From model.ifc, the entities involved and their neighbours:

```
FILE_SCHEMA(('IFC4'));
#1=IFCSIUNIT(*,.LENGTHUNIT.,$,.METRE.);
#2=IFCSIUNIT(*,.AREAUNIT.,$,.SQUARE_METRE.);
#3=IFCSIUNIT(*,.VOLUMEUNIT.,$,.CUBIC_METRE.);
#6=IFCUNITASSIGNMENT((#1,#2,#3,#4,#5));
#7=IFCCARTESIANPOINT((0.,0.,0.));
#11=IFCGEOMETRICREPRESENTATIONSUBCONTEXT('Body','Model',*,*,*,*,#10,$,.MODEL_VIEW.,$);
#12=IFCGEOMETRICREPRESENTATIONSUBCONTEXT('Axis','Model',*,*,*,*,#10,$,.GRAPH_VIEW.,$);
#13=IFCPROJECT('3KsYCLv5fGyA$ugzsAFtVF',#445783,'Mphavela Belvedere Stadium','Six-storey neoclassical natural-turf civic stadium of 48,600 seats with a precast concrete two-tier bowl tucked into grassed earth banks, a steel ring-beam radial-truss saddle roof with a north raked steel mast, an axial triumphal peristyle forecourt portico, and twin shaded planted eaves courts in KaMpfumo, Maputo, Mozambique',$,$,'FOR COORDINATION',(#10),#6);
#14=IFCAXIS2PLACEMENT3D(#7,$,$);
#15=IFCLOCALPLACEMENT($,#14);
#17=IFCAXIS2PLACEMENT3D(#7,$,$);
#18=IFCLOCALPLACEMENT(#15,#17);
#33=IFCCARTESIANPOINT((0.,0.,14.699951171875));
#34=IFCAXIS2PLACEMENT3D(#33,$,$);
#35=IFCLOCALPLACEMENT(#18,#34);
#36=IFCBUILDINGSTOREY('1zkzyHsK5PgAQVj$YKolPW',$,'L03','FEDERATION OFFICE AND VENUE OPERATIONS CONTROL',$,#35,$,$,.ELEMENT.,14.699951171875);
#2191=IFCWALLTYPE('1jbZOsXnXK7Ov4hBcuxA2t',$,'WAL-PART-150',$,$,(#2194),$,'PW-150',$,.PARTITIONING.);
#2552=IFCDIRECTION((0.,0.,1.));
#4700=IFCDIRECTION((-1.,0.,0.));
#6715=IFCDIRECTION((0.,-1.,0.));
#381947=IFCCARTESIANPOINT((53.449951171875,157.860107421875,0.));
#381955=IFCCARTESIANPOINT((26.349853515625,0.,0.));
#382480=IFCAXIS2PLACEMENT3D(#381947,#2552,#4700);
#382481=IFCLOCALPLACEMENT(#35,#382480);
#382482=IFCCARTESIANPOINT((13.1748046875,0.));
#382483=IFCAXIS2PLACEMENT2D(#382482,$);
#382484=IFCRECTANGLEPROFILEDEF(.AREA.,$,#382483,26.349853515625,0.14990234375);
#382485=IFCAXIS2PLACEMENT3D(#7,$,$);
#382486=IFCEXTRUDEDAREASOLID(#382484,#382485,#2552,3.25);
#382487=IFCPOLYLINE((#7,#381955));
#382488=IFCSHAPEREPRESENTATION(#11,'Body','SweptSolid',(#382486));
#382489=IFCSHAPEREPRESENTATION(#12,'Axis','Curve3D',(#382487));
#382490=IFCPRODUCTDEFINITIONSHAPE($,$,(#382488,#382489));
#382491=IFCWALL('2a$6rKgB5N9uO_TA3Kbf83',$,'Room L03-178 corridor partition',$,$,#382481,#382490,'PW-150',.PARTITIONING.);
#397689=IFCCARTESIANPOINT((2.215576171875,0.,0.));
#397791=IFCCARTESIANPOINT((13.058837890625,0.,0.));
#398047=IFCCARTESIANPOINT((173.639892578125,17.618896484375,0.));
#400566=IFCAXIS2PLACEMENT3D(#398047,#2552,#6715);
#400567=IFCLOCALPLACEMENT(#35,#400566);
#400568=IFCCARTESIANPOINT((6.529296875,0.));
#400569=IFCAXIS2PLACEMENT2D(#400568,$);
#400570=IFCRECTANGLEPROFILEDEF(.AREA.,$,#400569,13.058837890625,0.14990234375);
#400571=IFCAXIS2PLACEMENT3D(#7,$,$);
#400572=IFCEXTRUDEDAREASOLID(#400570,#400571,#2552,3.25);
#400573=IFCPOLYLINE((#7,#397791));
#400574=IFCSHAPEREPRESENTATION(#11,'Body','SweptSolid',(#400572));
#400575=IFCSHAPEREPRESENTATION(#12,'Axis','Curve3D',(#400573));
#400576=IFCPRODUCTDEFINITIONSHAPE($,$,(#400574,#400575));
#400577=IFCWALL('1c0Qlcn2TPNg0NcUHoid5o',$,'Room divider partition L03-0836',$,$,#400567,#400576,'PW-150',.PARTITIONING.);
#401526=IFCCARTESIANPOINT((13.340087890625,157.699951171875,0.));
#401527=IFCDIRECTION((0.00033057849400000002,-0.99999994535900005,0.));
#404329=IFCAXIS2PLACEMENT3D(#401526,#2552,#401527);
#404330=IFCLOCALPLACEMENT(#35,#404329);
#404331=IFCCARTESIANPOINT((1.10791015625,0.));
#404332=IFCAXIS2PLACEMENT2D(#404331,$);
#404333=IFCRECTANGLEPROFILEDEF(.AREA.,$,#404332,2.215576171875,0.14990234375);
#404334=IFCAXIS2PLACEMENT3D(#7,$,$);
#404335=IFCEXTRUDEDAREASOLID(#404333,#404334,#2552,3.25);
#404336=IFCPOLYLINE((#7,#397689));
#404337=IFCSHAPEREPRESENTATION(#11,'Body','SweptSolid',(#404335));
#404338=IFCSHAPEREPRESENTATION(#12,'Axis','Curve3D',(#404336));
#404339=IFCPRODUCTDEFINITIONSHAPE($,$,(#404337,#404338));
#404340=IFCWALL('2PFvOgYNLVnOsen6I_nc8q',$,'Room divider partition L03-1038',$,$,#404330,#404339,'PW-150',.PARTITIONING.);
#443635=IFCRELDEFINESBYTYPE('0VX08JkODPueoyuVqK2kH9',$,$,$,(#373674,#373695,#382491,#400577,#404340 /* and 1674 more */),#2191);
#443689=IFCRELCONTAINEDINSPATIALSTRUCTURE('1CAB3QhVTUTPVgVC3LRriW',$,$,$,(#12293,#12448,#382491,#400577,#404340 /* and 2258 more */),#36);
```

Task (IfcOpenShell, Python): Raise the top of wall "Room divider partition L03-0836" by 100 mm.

```python
import ifcopenshell
import ifcopenshell.geom
import ifcopenshell.util.representation
import ifcopenshell.util.shape
import ifcopenshell.util.unit

model = ifcopenshell.open("model.ifc")
unit_scale = ifcopenshell.util.unit.calculate_unit_scale(model)
settings = ifcopenshell.geom.settings()


def volume(element):
    """Net volume in cubic metres, openings subtracted."""
    shape = ifcopenshell.geom.create_shape(settings, element)
    return ifcopenshell.util.shape.get_volume(shape.geometry)


wall = model.by_id(400577)
before = volume(wall)

body = ifcopenshell.util.representation.get_representation(wall, "Model", "Body")
solid = body.Items[0]
old_height = solid.Depth
solid.Depth += 0.1 / unit_scale
after = volume(wall)

print(f"height {old_height:g} -> {solid.Depth:g}, volume {before:.3f} -> {after:.3f} m3")

model.write("model_updated.ifc")
```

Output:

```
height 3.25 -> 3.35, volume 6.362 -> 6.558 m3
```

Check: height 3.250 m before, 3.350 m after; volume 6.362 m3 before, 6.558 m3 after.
